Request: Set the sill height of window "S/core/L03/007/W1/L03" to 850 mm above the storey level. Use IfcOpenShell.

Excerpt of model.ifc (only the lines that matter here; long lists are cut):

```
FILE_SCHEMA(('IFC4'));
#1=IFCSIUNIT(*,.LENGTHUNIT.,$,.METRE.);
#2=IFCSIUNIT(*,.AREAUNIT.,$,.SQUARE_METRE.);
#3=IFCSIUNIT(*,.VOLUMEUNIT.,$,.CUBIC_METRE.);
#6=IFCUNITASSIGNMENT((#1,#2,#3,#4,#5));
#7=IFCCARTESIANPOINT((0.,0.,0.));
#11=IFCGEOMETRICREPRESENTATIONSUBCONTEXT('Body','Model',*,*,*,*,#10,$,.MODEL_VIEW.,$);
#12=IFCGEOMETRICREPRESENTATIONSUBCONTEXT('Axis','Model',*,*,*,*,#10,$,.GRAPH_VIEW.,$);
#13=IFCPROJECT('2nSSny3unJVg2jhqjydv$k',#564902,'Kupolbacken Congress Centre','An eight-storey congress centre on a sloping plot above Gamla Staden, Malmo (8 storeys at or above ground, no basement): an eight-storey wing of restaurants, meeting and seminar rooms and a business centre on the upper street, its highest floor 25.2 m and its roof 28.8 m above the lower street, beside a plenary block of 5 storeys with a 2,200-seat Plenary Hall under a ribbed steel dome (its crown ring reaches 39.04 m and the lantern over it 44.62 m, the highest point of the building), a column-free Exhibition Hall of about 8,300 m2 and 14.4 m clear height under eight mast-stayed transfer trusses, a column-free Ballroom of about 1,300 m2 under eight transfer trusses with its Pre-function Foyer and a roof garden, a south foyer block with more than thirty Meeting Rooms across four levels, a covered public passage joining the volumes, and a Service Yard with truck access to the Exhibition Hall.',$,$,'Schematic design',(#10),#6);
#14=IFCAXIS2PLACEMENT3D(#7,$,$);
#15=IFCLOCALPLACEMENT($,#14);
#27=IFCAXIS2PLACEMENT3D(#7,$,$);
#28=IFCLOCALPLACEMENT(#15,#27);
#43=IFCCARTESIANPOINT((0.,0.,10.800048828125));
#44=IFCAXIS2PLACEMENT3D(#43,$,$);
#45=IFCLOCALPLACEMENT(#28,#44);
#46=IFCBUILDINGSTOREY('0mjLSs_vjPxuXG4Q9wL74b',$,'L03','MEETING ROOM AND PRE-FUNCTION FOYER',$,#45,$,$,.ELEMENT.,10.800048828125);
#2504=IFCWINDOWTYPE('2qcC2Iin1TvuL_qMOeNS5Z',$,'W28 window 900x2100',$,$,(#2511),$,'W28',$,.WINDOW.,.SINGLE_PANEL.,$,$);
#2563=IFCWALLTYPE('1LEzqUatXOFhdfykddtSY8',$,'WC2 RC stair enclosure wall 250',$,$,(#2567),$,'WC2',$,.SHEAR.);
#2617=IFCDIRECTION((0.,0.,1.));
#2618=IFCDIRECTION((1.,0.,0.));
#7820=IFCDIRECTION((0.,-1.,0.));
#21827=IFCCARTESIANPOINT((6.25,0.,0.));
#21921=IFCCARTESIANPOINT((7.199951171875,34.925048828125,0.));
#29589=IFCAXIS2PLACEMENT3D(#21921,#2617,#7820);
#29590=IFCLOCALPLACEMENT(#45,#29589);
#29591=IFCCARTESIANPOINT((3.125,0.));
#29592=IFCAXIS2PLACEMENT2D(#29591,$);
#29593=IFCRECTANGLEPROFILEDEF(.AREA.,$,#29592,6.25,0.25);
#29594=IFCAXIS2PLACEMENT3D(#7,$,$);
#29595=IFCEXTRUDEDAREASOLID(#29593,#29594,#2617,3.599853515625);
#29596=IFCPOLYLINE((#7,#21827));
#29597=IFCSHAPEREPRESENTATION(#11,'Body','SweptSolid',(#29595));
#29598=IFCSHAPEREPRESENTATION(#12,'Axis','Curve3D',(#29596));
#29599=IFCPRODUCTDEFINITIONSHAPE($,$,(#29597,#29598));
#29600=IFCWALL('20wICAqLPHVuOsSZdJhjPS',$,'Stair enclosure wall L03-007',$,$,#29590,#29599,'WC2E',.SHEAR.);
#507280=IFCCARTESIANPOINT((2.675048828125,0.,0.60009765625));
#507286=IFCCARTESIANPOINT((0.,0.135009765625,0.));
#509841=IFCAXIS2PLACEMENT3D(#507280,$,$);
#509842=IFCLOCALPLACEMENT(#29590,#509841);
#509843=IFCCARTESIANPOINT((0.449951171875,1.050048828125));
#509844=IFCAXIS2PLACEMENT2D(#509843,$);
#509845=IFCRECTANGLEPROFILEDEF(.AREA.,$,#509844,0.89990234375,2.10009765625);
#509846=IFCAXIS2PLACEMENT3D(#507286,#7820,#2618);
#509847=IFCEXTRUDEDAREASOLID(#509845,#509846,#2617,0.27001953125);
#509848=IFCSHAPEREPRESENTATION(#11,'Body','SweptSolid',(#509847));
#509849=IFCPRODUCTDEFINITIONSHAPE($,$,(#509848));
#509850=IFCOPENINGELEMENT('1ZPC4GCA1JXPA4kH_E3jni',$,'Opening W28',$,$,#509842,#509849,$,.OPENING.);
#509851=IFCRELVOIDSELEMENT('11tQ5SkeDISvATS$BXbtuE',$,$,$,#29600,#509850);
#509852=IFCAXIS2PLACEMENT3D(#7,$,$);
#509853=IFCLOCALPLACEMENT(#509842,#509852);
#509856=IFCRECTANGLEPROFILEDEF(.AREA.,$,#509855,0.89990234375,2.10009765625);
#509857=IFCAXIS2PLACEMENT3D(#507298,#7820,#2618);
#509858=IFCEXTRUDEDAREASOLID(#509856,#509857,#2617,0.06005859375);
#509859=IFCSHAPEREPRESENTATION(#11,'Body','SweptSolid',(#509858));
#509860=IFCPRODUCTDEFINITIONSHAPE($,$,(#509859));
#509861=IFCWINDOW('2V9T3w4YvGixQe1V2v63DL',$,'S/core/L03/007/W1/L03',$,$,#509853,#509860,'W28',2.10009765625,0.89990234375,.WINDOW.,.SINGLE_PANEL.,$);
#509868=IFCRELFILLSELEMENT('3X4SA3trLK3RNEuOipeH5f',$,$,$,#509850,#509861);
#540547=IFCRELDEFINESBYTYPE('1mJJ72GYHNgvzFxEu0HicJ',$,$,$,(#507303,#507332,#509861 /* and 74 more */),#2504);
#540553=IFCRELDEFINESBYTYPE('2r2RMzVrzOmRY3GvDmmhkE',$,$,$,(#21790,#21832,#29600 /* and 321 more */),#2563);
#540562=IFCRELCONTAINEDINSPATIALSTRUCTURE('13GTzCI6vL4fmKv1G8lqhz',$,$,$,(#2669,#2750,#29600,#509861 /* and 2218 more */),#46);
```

```python
import numpy as np
import ifcopenshell
import ifcopenshell.api.geometry
import ifcopenshell.geom
import ifcopenshell.util.element
import ifcopenshell.util.placement
import ifcopenshell.util.shape
import ifcopenshell.util.unit

model = ifcopenshell.open("model.ifc")
unit_scale = ifcopenshell.util.unit.calculate_unit_scale(model)

window = model.by_guid("2V9T3w4YvGixQe1V2v63DL")
opening = window.FillsVoids[0].RelatingOpeningElement
storey = ifcopenshell.util.element.get_container(window, ifc_class="IfcBuildingStorey")
level = ifcopenshell.util.placement.get_local_placement(storey.ObjectPlacement)[2, 3]

# The opening's origin need not be at the sill, so measure its lowest point.
shape = ifcopenshell.geom.create_shape(ifcopenshell.geom.settings(), opening)
bottom = ifcopenshell.util.shape.get_shape_bottom_elevation(shape, shape.geometry) / unit_scale
dz = level + 0.85 - bottom

shift = np.array([0.0, 0.0, dz])
# The window is placed relative to its opening, so it follows when the opening moves.
matrix = ifcopenshell.util.placement.get_local_placement(opening.ObjectPlacement)
matrix[:3, 3] += shift
ifcopenshell.api.geometry.edit_object_placement(
    model, product=opening, matrix=matrix, is_si=False, should_transform_children=True
)

print(f"moved by {dz * unit_scale:+.3f} m")

model.write("model_updated.ifc")
```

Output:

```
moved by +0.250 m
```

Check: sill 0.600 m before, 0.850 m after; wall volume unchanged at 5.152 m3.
